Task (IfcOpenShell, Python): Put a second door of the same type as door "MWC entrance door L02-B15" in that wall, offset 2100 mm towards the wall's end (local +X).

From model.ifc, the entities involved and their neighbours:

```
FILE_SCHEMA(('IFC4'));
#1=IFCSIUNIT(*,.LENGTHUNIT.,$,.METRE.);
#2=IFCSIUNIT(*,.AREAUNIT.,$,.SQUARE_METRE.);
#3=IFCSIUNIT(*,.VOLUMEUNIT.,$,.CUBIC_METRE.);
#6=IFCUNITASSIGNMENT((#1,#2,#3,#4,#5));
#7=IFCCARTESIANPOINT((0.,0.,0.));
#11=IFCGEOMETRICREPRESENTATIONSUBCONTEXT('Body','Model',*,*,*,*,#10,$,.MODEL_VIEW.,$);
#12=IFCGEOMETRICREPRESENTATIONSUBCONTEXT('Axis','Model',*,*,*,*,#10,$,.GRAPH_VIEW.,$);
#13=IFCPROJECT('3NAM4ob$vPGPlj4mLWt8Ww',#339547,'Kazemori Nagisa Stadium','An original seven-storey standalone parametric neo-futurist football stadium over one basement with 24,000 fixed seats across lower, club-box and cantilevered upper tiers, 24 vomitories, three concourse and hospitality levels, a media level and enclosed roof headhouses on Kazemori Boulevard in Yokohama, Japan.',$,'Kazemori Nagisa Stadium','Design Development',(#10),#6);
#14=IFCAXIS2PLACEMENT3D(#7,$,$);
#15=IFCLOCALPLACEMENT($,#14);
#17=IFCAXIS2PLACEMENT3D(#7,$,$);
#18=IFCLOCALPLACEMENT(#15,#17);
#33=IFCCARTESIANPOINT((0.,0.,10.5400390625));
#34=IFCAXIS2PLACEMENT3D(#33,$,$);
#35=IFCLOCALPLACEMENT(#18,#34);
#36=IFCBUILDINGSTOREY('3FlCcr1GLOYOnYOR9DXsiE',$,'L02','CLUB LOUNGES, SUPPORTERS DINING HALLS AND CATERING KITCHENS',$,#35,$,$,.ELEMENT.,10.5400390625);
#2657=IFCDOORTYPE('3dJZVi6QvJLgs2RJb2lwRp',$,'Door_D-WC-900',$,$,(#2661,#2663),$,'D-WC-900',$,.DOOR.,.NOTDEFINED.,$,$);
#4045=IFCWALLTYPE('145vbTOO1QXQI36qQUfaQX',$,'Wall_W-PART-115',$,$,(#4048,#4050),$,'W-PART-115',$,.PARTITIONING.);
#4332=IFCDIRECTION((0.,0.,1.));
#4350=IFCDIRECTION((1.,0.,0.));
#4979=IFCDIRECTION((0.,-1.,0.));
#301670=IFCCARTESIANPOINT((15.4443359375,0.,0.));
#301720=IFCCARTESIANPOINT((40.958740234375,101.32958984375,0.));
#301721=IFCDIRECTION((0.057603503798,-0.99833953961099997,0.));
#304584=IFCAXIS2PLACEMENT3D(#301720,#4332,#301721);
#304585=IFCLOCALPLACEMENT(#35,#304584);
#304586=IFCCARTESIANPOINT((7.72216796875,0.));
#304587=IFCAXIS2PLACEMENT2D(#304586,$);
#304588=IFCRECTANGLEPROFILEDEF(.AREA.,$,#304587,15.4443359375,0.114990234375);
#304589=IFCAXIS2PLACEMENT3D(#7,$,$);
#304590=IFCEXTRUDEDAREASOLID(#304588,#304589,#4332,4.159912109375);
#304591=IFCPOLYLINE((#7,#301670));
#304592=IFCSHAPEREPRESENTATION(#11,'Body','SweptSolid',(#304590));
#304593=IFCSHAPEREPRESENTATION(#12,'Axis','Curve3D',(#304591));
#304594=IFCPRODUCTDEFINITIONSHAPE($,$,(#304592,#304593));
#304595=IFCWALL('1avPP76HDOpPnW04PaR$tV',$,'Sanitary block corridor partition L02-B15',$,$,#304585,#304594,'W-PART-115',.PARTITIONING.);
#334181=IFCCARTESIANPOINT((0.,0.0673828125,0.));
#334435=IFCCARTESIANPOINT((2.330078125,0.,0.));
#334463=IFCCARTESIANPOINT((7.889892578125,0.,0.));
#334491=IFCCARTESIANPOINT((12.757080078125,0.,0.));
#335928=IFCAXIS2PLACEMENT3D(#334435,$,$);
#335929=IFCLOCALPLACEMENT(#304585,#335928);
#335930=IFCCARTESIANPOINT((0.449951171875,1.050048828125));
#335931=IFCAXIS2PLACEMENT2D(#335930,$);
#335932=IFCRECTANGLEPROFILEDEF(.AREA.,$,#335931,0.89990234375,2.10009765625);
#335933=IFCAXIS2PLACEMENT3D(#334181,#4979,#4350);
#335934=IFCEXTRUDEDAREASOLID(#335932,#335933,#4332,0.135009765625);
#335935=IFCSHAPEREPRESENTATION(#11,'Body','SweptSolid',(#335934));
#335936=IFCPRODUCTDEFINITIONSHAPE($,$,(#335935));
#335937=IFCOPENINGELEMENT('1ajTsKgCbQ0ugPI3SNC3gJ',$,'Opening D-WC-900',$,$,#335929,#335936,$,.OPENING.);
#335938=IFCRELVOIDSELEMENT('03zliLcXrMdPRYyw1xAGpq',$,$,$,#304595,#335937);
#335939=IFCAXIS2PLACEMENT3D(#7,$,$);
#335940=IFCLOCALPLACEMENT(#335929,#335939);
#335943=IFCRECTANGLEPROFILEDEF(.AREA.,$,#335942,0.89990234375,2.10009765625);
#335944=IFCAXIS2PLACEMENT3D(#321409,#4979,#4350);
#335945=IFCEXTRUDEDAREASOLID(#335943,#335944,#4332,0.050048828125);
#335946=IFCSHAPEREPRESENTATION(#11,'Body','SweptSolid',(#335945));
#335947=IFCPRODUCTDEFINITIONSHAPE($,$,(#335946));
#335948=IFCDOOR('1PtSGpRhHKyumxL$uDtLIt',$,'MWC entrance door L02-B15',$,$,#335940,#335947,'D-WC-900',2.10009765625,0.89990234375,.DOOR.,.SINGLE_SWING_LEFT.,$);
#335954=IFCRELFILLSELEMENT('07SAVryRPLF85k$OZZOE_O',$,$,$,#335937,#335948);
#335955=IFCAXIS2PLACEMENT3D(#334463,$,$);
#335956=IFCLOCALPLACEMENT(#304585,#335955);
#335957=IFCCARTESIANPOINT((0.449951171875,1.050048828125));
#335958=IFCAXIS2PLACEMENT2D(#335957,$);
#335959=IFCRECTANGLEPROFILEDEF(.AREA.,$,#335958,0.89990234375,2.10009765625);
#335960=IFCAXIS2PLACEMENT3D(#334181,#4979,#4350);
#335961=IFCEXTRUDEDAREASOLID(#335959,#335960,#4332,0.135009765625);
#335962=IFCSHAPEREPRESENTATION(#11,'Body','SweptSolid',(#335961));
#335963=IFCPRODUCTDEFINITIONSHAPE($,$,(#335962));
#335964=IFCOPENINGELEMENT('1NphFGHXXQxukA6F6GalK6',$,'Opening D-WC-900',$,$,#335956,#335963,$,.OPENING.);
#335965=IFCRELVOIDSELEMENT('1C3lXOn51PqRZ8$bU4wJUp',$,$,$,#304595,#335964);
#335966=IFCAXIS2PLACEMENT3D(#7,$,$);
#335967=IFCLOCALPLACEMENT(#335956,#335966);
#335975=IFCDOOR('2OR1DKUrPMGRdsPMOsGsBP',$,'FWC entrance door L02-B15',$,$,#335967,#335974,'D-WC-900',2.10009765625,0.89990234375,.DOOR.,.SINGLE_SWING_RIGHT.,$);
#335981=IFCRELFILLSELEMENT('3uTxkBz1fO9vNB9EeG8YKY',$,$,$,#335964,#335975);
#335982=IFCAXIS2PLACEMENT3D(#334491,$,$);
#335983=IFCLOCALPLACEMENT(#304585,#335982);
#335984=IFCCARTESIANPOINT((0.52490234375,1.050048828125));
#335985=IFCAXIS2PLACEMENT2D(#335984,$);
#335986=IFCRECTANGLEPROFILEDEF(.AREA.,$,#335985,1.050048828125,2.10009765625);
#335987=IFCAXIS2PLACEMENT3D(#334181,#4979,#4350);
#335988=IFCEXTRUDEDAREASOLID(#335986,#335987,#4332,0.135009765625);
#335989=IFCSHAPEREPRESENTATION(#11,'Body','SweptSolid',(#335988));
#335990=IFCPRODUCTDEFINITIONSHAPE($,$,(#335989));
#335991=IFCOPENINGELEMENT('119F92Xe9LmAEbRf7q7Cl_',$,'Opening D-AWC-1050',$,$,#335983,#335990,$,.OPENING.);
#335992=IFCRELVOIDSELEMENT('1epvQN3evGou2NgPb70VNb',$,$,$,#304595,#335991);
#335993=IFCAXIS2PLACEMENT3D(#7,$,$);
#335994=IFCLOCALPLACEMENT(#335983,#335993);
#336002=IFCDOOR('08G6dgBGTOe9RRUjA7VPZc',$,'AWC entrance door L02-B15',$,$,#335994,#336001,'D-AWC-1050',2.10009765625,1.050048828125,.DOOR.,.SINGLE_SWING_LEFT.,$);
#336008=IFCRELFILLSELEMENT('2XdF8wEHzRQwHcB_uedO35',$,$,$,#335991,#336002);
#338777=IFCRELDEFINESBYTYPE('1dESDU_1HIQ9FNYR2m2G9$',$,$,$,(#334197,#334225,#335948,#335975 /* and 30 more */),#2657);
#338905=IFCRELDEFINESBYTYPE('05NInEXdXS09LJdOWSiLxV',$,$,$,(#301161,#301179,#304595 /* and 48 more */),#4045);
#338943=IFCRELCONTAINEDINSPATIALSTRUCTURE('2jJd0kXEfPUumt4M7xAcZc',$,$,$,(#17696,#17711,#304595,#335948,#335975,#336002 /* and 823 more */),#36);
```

```python
import ifcopenshell
import ifcopenshell.api.feature
import ifcopenshell.api.geometry
import ifcopenshell.api.root
import ifcopenshell.geom
import ifcopenshell.util.element
import ifcopenshell.util.placement
import ifcopenshell.util.shape

model = ifcopenshell.open("model.ifc")
settings = ifcopenshell.geom.settings()


def volume(element):
    """Net volume in cubic metres, openings subtracted."""
    shape = ifcopenshell.geom.create_shape(settings, element)
    return ifcopenshell.util.shape.get_volume(shape.geometry)


door = model.by_id(335948)
opening = door.FillsVoids[0].RelatingOpeningElement
wall = opening.VoidsElements[0].RelatingBuildingElement
before = volume(wall)
shift = ifcopenshell.util.placement.get_local_placement(wall.ObjectPlacement)[:3, 0] * 2.1

# copy_class copies the void relationship, type, container and properties, but no geometry.
new_opening = ifcopenshell.api.root.copy_class(model, product=opening)
new_opening.Representation = ifcopenshell.util.element.copy_deep(
    model, opening.Representation, exclude=["IfcGeometricRepresentationContext", "IfcRepresentationMap"]
)
new_door = ifcopenshell.api.root.copy_class(model, product=door)
new_door.Representation = ifcopenshell.util.element.copy_deep(
    model, door.Representation, exclude=["IfcGeometricRepresentationContext", "IfcRepresentationMap"]
)
new_door.Tag = None
ifcopenshell.api.feature.add_filling(model, opening=new_opening, element=new_door)

for old, new in ((opening, new_opening), (door, new_door)):
    matrix = ifcopenshell.util.placement.get_local_placement(old.ObjectPlacement)
    matrix[:3, 3] += shift
    ifcopenshell.api.geometry.edit_object_placement(model, product=new, matrix=matrix, is_si=False)

after = volume(wall)

print(f"wall volume {before:.3f} -> {after:.3f} m3")

model.write("model-out.ifc")
```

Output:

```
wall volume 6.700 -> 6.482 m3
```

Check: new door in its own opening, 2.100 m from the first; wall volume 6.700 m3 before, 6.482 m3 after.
